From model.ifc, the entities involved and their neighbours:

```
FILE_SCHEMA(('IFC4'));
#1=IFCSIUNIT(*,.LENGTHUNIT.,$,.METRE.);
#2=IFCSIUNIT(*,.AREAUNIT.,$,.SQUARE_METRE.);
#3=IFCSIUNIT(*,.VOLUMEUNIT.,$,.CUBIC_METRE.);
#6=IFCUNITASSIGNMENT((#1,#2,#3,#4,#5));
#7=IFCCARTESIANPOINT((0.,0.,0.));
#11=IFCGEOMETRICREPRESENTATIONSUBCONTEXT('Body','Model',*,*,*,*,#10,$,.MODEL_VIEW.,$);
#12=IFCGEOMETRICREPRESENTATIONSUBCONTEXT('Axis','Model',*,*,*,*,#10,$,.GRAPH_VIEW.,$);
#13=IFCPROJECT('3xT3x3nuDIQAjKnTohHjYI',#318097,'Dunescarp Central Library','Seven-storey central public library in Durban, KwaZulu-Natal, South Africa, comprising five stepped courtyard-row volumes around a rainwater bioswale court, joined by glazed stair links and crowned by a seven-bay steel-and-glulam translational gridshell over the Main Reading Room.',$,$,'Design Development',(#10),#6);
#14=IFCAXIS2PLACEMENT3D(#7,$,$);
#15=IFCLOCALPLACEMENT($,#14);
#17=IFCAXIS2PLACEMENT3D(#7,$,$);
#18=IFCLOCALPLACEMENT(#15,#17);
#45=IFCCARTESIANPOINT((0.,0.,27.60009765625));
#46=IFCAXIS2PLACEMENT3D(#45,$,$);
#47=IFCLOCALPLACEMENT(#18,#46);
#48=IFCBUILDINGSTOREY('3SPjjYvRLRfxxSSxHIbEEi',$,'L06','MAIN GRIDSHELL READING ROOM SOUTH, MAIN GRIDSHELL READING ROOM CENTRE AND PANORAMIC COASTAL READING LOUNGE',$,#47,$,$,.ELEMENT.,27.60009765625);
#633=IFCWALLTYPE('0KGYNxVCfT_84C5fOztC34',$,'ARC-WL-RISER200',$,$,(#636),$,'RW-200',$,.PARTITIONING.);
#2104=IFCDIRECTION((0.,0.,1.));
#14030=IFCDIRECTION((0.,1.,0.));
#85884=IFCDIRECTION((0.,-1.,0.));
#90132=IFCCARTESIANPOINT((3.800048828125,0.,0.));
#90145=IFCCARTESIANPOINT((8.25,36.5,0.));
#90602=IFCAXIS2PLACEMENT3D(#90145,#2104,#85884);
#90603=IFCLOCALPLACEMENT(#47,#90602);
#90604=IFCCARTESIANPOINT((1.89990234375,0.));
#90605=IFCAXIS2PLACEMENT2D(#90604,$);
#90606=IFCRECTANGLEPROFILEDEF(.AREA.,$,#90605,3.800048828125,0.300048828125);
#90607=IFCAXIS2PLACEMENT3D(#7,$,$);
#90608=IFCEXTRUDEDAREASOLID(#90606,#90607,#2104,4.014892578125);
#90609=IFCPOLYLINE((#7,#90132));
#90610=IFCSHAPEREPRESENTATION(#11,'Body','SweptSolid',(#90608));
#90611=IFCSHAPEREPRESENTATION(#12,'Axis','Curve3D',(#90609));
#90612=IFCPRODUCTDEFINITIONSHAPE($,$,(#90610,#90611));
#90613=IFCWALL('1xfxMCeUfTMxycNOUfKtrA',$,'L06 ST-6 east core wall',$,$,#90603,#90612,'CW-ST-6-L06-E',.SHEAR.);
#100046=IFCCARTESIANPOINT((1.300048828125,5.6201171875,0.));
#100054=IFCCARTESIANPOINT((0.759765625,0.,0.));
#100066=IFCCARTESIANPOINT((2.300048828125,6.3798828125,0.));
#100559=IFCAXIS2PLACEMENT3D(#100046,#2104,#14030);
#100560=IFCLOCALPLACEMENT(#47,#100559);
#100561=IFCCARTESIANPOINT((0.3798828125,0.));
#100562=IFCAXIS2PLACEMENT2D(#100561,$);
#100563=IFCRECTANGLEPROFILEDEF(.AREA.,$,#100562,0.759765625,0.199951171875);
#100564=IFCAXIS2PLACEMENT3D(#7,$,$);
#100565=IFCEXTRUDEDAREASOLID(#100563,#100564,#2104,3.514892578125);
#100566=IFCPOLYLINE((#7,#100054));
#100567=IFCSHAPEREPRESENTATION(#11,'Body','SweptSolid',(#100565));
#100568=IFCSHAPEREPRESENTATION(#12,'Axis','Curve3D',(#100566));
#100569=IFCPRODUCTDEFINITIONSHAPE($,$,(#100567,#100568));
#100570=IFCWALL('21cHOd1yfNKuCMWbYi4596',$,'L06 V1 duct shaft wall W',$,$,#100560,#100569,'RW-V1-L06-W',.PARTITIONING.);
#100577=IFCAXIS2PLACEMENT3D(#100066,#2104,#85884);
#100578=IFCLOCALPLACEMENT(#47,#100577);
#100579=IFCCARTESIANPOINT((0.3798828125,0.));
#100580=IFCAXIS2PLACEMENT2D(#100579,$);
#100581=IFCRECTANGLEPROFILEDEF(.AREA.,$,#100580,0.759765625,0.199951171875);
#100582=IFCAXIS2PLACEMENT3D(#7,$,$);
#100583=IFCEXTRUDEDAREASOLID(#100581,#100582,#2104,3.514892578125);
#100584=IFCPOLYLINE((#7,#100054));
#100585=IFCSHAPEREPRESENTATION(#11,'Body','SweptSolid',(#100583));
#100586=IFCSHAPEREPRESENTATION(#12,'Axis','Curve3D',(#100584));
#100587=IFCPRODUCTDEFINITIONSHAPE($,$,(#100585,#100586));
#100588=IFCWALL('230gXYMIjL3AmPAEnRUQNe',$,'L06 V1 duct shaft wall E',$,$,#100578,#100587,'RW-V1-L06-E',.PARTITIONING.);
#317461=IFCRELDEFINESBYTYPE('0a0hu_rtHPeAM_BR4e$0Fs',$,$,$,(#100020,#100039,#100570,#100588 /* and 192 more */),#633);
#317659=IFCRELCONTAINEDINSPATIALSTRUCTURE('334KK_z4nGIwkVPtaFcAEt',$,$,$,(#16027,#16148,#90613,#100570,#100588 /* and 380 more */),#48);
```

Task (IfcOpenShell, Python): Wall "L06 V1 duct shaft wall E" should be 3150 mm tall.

```python
import ifcopenshell
import ifcopenshell.geom
import ifcopenshell.util.representation
import ifcopenshell.util.shape
import ifcopenshell.util.unit

model = ifcopenshell.open("model.ifc")
unit_scale = ifcopenshell.util.unit.calculate_unit_scale(model)
settings = ifcopenshell.geom.settings()


def volume(element):
    """Net volume in cubic metres, openings subtracted."""
    shape = ifcopenshell.geom.create_shape(settings, element)
    return ifcopenshell.util.shape.get_volume(shape.geometry)


wall = model.by_guid("230gXYMIjL3AmPAEnRUQNe")
before = volume(wall)

body = ifcopenshell.util.representation.get_representation(wall, "Model", "Body")
solid = body.Items[0]
old_height = solid.Depth
solid.Depth = 3.15 / unit_scale
after = volume(wall)

print(f"height {old_height:g} -> {solid.Depth:g}, volume {before:.3f} -> {after:.3f} m3")

model.write("model_updated.ifc")
```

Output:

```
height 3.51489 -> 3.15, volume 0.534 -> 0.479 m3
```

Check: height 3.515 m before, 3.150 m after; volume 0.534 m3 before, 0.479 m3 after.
